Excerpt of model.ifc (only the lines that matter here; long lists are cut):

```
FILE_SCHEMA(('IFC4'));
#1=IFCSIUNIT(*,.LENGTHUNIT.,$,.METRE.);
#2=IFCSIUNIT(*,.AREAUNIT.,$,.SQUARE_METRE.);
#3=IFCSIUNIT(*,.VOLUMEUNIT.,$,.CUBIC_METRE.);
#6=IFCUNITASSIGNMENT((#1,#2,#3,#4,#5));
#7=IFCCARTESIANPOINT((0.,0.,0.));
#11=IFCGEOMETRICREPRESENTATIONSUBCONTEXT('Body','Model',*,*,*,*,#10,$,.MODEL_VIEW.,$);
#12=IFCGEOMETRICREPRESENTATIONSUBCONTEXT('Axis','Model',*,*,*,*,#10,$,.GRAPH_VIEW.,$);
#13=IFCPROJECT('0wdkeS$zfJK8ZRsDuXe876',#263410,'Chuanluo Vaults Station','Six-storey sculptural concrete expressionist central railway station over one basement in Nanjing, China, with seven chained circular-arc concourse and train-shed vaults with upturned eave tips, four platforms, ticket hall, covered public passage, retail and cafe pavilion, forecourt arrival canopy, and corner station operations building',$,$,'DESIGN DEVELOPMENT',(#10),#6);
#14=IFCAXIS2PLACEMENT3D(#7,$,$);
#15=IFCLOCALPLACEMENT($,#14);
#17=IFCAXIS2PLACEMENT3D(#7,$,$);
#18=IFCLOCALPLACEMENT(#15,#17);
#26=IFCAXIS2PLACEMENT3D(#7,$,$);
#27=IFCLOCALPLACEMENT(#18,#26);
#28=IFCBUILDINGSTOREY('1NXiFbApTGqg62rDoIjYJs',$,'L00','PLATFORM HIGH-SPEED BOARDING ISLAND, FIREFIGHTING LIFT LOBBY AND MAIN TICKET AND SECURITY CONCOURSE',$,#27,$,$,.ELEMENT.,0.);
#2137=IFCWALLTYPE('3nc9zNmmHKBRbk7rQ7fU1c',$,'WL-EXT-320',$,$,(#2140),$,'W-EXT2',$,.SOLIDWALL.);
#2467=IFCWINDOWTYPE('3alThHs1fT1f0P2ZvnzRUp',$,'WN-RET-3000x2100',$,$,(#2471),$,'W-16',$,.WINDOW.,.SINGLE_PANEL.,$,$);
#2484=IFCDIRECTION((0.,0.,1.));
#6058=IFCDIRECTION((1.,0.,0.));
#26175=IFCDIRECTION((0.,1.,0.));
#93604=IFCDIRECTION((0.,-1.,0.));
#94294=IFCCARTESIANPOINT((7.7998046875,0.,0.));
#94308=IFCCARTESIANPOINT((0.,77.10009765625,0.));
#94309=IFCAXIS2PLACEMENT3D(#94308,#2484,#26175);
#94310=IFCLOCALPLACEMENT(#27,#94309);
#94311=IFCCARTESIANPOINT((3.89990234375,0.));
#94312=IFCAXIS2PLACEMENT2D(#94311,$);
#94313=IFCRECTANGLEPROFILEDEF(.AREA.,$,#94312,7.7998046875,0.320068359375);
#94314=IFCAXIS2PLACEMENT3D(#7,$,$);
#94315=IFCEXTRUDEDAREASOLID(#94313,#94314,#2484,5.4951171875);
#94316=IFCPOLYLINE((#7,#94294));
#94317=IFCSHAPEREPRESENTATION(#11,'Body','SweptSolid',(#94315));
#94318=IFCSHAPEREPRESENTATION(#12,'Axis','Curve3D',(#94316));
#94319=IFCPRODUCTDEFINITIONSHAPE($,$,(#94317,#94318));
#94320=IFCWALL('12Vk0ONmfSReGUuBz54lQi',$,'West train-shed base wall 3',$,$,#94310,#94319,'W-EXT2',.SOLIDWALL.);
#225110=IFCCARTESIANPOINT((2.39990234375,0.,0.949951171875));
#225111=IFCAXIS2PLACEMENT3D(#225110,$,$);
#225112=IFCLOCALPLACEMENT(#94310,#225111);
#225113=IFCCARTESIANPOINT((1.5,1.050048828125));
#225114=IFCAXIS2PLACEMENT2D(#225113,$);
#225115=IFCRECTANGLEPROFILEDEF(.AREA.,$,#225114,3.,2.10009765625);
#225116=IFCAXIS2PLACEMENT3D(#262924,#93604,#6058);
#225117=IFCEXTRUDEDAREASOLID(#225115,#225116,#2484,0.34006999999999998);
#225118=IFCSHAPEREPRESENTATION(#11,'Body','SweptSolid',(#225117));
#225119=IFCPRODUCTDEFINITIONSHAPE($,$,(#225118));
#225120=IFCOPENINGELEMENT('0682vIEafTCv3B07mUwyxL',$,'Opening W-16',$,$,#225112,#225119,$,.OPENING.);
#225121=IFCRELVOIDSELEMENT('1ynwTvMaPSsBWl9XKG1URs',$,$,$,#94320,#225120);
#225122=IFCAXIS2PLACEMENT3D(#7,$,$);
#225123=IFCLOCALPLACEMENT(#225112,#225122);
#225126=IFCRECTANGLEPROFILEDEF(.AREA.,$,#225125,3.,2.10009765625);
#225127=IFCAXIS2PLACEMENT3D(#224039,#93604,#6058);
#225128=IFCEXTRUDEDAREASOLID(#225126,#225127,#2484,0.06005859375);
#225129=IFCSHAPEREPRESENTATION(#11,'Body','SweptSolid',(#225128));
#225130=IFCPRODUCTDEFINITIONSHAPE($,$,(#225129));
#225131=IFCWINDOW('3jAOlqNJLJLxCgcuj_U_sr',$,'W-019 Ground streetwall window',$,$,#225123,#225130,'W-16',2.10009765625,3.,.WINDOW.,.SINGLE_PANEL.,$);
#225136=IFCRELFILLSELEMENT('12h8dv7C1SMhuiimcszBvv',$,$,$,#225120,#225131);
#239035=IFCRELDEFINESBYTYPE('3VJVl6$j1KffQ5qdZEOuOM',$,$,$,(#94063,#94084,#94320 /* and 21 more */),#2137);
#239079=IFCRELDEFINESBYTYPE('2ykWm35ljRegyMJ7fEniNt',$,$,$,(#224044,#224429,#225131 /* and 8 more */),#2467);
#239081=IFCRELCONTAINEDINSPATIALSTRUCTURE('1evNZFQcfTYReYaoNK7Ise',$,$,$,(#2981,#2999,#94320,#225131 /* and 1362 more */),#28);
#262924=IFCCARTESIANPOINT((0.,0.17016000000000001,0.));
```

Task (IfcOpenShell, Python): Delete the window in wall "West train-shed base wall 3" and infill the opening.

```python
import ifcopenshell
import ifcopenshell.api.feature
import ifcopenshell.api.root
import ifcopenshell.geom
import ifcopenshell.util.shape

model = ifcopenshell.open("model.ifc")
settings = ifcopenshell.geom.settings()


def volume(element):
    """Net volume in cubic metres, openings subtracted."""
    shape = ifcopenshell.geom.create_shape(settings, element)
    return ifcopenshell.util.shape.get_volume(shape.geometry)


window = model.by_guid("3jAOlqNJLJLxCgcuj_U_sr")
opening = window.FillsVoids[0].RelatingOpeningElement
wall = opening.VoidsElements[0].RelatingBuildingElement
before = volume(wall)

ifcopenshell.api.root.remove_product(model, product=window)
ifcopenshell.api.feature.remove_feature(model, feature=opening)

after = volume(wall)

print(f"wall volume {before:.3f} -> {after:.3f} m3")

model.write("model-out.ifc")
```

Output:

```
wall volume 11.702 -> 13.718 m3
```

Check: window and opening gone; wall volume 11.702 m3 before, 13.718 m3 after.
